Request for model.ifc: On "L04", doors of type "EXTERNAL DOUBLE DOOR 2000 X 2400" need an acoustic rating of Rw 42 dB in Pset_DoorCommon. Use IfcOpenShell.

First a look at what the model holds.

```python
import ifcopenshell
import ifcopenshell.util.element

model = ifcopenshell.open("model.ifc")
print(model.schema)
storey = next(s for s in model.by_type("IfcBuildingStorey") if s.Name == "L04")
doors = [e for e in ifcopenshell.util.element.get_decomposition(storey) if e.is_a("IfcDoor")]
seen = {}
for e in doors:
    element_type = ifcopenshell.util.element.get_type(e)
    key = (element_type.Name if element_type != e and element_type else None, ifcopenshell.util.element.get_pset(e, "Pset_DoorCommon", "AcousticRating"))
    seen[key] = seen.get(key, 0) + 1
for (name, value), count in sorted(seen.items(), key=str):
    print(count, "x", name, "|", value)
```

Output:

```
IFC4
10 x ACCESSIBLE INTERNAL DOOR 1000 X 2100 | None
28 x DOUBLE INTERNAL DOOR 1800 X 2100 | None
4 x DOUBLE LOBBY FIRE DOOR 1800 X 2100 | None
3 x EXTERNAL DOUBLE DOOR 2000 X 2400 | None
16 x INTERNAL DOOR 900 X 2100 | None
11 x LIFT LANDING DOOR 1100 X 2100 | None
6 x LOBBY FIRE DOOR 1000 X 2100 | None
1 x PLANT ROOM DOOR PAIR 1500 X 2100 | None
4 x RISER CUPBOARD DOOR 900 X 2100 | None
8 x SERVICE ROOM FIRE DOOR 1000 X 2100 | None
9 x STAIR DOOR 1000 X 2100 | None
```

```python
import ifcopenshell
import ifcopenshell.api.pset
import ifcopenshell.util.element

model = ifcopenshell.open("model.ifc")

storey = next(s for s in model.by_type("IfcBuildingStorey") if s.Name == "L04")
doors = [e for e in ifcopenshell.util.element.get_decomposition(storey) if e.is_a("IfcDoor")]

count = 0
for e in doors:
    element_type = ifcopenshell.util.element.get_type(e)
    if element_type in (None, e) or element_type.Name != "EXTERNAL DOUBLE DOOR 2000 X 2400":
        continue
    found = ifcopenshell.util.element.get_pset(e, "Pset_DoorCommon", should_inherit=False)
    if found:
        pset = model.by_id(found["id"])
        if len(ifcopenshell.util.element.get_elements_by_pset(pset)) > 1:
            pset = ifcopenshell.api.pset.unshare_pset(model, products=[e], pset=pset)[0]
    else:
        pset = ifcopenshell.api.pset.add_pset(model, product=e, name="Pset_DoorCommon")
    ifcopenshell.api.pset.edit_pset(model, pset=pset, properties={"AcousticRating": "Rw 42 dB"})
    count += 1

print(count, "doors updated")

model.write("model_updated.ifc")
```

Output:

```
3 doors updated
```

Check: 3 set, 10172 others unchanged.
